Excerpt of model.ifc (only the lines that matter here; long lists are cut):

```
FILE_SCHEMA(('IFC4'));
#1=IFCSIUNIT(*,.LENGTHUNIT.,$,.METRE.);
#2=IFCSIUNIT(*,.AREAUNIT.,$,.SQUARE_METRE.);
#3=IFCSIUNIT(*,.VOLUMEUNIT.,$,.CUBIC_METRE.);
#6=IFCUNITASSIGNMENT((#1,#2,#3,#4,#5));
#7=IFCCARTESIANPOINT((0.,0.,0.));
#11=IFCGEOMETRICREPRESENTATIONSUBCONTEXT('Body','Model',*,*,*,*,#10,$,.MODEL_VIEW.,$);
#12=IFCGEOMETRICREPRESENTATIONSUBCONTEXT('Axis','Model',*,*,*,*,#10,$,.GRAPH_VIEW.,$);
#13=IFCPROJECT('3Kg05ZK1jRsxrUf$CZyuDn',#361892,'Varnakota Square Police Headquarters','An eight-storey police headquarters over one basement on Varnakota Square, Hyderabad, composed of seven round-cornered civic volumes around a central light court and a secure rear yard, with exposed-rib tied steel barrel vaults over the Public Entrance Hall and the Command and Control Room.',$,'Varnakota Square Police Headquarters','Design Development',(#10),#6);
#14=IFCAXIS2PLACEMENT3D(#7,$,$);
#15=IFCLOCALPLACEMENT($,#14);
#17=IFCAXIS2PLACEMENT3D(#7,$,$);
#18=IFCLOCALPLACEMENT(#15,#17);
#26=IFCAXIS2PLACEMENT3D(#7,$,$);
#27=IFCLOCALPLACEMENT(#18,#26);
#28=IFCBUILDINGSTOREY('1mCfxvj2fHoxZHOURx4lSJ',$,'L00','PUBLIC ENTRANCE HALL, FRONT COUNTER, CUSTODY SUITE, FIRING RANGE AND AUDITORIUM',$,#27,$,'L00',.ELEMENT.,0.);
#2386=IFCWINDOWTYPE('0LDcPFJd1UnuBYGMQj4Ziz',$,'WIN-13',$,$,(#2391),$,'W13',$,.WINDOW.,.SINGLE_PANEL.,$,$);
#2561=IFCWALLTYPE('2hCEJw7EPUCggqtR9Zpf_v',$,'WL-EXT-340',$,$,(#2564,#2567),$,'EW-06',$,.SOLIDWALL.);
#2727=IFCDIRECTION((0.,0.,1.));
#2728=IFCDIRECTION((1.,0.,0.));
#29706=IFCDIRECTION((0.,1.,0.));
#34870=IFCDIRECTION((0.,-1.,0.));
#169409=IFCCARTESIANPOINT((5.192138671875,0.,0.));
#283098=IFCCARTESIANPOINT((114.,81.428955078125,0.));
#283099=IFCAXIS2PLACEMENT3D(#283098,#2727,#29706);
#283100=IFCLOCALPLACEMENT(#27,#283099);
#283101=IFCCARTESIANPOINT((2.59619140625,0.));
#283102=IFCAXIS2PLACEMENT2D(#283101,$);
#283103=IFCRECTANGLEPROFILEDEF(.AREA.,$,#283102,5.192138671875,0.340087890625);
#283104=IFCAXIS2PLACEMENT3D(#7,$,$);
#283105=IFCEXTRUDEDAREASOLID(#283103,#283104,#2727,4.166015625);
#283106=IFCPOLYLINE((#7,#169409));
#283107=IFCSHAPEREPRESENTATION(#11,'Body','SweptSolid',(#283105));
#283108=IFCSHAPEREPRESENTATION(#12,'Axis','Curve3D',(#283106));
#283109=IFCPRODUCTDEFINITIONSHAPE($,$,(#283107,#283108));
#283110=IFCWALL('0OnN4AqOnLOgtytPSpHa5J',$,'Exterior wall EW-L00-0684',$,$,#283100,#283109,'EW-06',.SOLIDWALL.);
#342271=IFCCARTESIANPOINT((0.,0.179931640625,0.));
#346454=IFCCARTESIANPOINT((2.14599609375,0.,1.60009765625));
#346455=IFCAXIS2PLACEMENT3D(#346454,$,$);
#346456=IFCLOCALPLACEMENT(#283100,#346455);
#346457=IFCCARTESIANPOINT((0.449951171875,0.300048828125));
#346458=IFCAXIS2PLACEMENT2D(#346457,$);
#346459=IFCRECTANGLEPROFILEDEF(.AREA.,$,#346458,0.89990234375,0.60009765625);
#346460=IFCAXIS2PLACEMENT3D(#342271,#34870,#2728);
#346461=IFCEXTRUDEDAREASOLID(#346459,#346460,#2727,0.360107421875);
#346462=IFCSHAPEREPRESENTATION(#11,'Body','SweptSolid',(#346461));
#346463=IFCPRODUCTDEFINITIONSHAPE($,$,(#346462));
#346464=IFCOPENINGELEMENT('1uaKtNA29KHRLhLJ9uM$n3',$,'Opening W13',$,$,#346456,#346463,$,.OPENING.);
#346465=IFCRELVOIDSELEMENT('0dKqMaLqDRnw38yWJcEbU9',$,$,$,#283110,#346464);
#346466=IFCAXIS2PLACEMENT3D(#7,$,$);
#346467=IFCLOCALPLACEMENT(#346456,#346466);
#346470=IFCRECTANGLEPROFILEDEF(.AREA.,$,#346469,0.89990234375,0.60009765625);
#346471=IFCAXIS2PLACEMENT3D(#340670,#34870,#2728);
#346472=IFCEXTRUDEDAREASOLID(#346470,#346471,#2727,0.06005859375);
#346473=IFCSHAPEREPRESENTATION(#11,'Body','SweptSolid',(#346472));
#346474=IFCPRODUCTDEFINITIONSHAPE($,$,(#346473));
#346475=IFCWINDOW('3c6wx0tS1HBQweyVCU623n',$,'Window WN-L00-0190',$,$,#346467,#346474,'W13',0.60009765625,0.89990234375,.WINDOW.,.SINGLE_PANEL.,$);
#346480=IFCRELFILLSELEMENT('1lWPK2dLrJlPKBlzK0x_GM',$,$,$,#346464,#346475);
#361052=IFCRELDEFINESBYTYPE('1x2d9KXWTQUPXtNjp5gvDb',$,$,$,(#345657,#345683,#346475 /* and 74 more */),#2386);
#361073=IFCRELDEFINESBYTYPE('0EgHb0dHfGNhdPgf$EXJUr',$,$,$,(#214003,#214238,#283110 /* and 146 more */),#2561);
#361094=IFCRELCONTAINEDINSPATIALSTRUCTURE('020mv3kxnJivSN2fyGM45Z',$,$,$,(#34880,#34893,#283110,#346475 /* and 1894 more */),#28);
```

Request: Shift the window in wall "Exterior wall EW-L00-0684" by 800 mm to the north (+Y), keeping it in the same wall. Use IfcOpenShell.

```python
import ifcopenshell
import ifcopenshell.api.geometry
import ifcopenshell.util.placement

model = ifcopenshell.open("model.ifc")

window = model.by_guid("3c6wx0tS1HBQweyVCU623n")
opening = window.FillsVoids[0].RelatingOpeningElement
wall = opening.VoidsElements[0].RelatingBuildingElement

wall_matrix = ifcopenshell.util.placement.get_local_placement(wall.ObjectPlacement)
shift = wall_matrix[:3, 0] * 0.8
before = ifcopenshell.util.placement.get_local_placement(window.ObjectPlacement)[:3, 3].copy()

# The window is placed relative to its opening, so it follows when the opening moves.
matrix = ifcopenshell.util.placement.get_local_placement(opening.ObjectPlacement)
matrix[:3, 3] += shift
ifcopenshell.api.geometry.edit_object_placement(
    model, product=opening, matrix=matrix, is_si=False, should_transform_children=True
)

after = ifcopenshell.util.placement.get_local_placement(window.ObjectPlacement)[:3, 3]
print("window moved by", (after - before).round(3) + 0.0)

model.write("model_rev.ifc")
```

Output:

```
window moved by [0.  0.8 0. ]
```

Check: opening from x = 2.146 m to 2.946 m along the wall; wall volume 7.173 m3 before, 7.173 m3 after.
